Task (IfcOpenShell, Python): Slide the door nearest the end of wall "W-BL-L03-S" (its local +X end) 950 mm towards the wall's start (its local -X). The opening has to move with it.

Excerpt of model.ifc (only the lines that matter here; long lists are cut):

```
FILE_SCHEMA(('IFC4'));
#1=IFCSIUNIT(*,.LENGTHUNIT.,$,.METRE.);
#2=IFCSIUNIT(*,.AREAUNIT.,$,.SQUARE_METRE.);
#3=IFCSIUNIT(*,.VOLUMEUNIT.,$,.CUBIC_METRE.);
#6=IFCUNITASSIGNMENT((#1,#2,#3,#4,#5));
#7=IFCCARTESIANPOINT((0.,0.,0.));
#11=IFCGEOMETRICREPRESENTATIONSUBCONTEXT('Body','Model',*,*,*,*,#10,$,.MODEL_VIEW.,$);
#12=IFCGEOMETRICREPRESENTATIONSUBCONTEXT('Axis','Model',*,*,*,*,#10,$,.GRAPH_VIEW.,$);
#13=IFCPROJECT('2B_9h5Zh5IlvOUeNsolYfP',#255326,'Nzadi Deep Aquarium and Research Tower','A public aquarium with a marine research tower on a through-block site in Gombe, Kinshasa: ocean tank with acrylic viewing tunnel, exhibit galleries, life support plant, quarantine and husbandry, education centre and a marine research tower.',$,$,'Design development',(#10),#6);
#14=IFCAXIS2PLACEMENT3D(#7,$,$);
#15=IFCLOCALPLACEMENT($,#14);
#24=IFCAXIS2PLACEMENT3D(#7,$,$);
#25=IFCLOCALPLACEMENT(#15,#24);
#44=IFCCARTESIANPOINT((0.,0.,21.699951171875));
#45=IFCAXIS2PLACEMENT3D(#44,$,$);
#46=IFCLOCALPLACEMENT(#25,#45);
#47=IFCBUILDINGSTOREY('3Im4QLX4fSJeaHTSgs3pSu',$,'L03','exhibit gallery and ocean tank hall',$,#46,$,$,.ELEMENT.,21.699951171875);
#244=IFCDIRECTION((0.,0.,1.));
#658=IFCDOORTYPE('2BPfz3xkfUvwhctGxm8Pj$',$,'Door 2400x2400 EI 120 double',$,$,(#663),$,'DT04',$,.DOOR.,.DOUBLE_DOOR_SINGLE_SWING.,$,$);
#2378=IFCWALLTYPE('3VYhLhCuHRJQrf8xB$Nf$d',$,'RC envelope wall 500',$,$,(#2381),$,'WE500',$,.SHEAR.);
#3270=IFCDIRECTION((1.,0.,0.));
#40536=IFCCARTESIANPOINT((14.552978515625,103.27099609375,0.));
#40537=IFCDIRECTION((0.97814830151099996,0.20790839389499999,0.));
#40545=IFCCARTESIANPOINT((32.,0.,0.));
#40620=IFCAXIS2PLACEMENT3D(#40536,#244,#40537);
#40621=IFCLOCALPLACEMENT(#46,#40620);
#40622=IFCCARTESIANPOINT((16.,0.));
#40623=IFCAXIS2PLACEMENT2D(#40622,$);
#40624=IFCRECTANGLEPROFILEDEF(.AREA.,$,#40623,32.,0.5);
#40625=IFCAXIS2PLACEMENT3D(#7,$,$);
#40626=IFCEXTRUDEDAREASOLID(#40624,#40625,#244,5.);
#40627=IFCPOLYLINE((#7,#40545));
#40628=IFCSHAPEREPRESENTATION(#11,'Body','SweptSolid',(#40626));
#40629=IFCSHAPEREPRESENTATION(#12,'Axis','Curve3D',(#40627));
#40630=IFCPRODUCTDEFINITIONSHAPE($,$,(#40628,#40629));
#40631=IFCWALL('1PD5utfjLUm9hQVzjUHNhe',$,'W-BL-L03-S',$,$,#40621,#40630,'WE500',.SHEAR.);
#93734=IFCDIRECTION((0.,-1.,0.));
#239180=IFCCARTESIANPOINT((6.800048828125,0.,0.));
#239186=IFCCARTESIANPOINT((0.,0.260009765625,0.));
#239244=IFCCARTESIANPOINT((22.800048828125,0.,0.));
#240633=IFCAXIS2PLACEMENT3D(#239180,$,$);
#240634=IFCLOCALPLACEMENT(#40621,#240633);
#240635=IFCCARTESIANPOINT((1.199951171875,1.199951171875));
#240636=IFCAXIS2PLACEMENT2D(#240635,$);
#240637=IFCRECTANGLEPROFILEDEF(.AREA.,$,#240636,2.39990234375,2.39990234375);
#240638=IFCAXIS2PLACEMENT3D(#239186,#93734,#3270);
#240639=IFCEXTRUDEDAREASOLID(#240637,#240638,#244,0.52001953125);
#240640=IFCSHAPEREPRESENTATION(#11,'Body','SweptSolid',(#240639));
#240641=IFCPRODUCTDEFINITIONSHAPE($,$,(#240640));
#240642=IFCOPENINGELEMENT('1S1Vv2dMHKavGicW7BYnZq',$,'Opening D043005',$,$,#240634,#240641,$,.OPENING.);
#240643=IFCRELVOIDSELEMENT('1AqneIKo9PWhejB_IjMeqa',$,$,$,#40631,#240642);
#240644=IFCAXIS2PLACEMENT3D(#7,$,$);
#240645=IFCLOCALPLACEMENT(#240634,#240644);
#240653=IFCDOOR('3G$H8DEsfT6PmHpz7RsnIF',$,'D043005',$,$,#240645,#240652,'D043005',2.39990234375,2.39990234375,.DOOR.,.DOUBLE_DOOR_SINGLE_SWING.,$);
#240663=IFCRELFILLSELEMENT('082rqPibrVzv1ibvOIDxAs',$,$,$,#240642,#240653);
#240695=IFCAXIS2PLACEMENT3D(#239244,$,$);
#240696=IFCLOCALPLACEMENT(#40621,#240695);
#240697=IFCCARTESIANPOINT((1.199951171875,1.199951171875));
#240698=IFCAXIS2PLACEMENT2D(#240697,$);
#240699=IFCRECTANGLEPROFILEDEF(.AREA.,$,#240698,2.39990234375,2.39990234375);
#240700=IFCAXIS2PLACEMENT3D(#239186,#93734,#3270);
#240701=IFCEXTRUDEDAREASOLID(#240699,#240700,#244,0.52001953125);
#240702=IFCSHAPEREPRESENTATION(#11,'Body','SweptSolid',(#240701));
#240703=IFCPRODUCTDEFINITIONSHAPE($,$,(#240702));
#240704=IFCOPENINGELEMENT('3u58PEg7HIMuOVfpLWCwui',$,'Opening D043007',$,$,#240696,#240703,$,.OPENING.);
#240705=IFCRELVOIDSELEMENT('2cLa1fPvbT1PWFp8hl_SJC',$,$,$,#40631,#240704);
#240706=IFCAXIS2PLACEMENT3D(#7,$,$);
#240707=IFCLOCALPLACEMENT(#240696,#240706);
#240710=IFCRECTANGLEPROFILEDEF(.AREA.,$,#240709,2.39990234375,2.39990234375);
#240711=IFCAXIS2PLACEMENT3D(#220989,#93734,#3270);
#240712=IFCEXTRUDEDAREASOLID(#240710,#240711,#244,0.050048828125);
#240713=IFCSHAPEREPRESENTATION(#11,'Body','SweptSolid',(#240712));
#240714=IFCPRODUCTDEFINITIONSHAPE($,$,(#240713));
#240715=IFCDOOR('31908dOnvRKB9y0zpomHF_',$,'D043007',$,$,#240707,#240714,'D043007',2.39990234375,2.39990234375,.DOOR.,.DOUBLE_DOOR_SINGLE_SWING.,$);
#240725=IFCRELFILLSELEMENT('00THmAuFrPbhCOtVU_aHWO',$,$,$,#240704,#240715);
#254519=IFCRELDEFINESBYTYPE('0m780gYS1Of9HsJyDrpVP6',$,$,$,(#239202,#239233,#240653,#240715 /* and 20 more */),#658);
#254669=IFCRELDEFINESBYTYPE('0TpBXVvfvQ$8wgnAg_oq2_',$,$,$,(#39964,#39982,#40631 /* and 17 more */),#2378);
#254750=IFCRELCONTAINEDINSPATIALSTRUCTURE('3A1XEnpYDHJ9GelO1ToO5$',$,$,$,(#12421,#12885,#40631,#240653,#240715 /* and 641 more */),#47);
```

```python
import ifcopenshell
import ifcopenshell.api.geometry
import ifcopenshell.util.placement

model = ifcopenshell.open("model.ifc")

door = model.by_id(240715)
opening = door.FillsVoids[0].RelatingOpeningElement
wall = opening.VoidsElements[0].RelatingBuildingElement

wall_matrix = ifcopenshell.util.placement.get_local_placement(wall.ObjectPlacement)
shift = wall_matrix[:3, 0] * -0.95
before = ifcopenshell.util.placement.get_local_placement(door.ObjectPlacement)[:3, 3].copy()

# The door is placed relative to its opening, so it follows when the opening moves.
matrix = ifcopenshell.util.placement.get_local_placement(opening.ObjectPlacement)
matrix[:3, 3] += shift
ifcopenshell.api.geometry.edit_object_placement(
    model, product=opening, matrix=matrix, is_si=False, should_transform_children=True
)

after = ifcopenshell.util.placement.get_local_placement(door.ObjectPlacement)[:3, 3]
print("door moved by", (after - before).round(3) + 0.0)

model.write("model_v2.ifc")
```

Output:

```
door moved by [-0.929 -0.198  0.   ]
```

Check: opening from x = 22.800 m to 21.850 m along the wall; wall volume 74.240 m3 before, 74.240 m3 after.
